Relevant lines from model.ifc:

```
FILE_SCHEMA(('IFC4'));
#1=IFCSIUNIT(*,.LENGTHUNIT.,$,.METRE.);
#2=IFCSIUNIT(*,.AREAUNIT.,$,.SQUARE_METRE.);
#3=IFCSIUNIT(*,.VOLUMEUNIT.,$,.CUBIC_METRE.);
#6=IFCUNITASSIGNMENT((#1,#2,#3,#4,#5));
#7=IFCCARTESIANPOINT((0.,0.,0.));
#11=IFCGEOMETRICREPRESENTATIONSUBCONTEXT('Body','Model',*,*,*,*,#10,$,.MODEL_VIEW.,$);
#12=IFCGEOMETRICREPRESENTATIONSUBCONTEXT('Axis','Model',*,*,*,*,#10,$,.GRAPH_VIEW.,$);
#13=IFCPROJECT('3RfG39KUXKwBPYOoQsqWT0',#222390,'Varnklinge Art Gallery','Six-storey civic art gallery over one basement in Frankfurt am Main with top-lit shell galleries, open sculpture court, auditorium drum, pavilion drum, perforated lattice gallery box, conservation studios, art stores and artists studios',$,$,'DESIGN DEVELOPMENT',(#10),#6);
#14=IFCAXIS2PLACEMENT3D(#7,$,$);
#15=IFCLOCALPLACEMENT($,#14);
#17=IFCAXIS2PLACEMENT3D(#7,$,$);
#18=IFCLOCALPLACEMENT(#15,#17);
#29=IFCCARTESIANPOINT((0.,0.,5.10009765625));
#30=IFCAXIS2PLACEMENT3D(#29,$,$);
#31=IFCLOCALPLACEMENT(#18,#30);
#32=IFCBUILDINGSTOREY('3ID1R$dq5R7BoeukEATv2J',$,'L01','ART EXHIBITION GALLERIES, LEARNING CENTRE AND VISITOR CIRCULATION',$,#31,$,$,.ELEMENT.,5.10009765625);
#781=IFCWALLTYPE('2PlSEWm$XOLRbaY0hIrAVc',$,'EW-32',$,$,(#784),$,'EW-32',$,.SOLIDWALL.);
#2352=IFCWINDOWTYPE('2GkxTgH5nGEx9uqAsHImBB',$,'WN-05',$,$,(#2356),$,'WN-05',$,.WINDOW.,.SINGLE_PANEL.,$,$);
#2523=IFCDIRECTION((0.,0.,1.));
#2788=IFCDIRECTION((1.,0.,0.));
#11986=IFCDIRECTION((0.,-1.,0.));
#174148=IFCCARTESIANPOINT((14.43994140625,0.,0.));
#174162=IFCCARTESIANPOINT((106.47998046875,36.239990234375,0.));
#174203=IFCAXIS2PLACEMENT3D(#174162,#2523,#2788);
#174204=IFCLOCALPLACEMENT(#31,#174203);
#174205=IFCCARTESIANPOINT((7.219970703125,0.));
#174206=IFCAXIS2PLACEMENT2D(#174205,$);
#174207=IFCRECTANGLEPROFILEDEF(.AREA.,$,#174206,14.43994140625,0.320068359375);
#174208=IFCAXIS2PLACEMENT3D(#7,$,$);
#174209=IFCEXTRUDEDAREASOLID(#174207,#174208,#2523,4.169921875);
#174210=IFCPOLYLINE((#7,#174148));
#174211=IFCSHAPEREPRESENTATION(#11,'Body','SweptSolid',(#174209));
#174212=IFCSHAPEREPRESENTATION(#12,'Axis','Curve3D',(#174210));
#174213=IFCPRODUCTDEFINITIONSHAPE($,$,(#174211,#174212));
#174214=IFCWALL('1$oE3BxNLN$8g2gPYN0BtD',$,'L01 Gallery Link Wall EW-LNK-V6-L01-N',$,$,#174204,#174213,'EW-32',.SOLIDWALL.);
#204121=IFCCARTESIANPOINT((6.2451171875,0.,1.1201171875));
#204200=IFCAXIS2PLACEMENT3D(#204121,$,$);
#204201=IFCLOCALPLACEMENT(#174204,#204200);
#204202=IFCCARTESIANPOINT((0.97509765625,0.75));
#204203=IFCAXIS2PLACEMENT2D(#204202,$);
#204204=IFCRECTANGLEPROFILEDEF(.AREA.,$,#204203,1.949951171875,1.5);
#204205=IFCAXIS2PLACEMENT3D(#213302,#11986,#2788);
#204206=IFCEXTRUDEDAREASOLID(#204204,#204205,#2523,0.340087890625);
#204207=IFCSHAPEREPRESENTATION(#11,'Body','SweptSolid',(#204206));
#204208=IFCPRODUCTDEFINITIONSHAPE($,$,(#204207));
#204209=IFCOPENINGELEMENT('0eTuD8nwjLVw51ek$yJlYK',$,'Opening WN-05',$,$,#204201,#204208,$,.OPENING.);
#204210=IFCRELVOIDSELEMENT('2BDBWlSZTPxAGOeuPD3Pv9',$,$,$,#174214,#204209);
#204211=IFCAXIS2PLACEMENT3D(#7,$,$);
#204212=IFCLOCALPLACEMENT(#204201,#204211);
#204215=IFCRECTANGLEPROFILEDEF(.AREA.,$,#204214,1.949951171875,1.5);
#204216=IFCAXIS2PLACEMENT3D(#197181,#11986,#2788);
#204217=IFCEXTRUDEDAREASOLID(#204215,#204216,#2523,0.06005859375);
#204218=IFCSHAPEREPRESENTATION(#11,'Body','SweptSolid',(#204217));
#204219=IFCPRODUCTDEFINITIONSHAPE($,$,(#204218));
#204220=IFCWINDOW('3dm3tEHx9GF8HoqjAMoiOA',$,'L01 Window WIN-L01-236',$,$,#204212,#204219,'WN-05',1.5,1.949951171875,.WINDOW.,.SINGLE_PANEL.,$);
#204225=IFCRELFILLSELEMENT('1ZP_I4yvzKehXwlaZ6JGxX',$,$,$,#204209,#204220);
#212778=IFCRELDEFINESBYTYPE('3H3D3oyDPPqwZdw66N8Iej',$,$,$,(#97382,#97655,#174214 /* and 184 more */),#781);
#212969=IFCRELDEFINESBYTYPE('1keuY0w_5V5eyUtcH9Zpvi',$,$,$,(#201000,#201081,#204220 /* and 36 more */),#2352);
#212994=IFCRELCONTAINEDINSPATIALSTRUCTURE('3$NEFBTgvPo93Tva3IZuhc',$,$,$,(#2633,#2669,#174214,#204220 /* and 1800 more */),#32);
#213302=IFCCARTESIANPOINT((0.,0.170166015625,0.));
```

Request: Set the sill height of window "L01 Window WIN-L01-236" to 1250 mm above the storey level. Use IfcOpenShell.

```python
import numpy as np
import ifcopenshell
import ifcopenshell.api.geometry
import ifcopenshell.geom
import ifcopenshell.util.element
import ifcopenshell.util.placement
import ifcopenshell.util.shape
import ifcopenshell.util.unit

model = ifcopenshell.open("model.ifc")
unit_scale = ifcopenshell.util.unit.calculate_unit_scale(model)

window = model.by_id(204220)
opening = window.FillsVoids[0].RelatingOpeningElement
storey = ifcopenshell.util.element.get_container(window, ifc_class="IfcBuildingStorey")
level = ifcopenshell.util.placement.get_local_placement(storey.ObjectPlacement)[2, 3]

# The opening's origin need not be at the sill, so measure its lowest point.
shape = ifcopenshell.geom.create_shape(ifcopenshell.geom.settings(), opening)
bottom = ifcopenshell.util.shape.get_shape_bottom_elevation(shape, shape.geometry) / unit_scale
dz = level + 1.25 / unit_scale - bottom

shift = np.array([0.0, 0.0, dz])
# The window is placed relative to its opening, so it follows when the opening moves.
matrix = ifcopenshell.util.placement.get_local_placement(opening.ObjectPlacement)
matrix[:3, 3] += shift
ifcopenshell.api.geometry.edit_object_placement(
    model, product=opening, matrix=matrix, is_si=False, should_transform_children=True
)

print(f"moved by {dz * unit_scale:+.3f} m")

model.write("model_updated.ifc")
```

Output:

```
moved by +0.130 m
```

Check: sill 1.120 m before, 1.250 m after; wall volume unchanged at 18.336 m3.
